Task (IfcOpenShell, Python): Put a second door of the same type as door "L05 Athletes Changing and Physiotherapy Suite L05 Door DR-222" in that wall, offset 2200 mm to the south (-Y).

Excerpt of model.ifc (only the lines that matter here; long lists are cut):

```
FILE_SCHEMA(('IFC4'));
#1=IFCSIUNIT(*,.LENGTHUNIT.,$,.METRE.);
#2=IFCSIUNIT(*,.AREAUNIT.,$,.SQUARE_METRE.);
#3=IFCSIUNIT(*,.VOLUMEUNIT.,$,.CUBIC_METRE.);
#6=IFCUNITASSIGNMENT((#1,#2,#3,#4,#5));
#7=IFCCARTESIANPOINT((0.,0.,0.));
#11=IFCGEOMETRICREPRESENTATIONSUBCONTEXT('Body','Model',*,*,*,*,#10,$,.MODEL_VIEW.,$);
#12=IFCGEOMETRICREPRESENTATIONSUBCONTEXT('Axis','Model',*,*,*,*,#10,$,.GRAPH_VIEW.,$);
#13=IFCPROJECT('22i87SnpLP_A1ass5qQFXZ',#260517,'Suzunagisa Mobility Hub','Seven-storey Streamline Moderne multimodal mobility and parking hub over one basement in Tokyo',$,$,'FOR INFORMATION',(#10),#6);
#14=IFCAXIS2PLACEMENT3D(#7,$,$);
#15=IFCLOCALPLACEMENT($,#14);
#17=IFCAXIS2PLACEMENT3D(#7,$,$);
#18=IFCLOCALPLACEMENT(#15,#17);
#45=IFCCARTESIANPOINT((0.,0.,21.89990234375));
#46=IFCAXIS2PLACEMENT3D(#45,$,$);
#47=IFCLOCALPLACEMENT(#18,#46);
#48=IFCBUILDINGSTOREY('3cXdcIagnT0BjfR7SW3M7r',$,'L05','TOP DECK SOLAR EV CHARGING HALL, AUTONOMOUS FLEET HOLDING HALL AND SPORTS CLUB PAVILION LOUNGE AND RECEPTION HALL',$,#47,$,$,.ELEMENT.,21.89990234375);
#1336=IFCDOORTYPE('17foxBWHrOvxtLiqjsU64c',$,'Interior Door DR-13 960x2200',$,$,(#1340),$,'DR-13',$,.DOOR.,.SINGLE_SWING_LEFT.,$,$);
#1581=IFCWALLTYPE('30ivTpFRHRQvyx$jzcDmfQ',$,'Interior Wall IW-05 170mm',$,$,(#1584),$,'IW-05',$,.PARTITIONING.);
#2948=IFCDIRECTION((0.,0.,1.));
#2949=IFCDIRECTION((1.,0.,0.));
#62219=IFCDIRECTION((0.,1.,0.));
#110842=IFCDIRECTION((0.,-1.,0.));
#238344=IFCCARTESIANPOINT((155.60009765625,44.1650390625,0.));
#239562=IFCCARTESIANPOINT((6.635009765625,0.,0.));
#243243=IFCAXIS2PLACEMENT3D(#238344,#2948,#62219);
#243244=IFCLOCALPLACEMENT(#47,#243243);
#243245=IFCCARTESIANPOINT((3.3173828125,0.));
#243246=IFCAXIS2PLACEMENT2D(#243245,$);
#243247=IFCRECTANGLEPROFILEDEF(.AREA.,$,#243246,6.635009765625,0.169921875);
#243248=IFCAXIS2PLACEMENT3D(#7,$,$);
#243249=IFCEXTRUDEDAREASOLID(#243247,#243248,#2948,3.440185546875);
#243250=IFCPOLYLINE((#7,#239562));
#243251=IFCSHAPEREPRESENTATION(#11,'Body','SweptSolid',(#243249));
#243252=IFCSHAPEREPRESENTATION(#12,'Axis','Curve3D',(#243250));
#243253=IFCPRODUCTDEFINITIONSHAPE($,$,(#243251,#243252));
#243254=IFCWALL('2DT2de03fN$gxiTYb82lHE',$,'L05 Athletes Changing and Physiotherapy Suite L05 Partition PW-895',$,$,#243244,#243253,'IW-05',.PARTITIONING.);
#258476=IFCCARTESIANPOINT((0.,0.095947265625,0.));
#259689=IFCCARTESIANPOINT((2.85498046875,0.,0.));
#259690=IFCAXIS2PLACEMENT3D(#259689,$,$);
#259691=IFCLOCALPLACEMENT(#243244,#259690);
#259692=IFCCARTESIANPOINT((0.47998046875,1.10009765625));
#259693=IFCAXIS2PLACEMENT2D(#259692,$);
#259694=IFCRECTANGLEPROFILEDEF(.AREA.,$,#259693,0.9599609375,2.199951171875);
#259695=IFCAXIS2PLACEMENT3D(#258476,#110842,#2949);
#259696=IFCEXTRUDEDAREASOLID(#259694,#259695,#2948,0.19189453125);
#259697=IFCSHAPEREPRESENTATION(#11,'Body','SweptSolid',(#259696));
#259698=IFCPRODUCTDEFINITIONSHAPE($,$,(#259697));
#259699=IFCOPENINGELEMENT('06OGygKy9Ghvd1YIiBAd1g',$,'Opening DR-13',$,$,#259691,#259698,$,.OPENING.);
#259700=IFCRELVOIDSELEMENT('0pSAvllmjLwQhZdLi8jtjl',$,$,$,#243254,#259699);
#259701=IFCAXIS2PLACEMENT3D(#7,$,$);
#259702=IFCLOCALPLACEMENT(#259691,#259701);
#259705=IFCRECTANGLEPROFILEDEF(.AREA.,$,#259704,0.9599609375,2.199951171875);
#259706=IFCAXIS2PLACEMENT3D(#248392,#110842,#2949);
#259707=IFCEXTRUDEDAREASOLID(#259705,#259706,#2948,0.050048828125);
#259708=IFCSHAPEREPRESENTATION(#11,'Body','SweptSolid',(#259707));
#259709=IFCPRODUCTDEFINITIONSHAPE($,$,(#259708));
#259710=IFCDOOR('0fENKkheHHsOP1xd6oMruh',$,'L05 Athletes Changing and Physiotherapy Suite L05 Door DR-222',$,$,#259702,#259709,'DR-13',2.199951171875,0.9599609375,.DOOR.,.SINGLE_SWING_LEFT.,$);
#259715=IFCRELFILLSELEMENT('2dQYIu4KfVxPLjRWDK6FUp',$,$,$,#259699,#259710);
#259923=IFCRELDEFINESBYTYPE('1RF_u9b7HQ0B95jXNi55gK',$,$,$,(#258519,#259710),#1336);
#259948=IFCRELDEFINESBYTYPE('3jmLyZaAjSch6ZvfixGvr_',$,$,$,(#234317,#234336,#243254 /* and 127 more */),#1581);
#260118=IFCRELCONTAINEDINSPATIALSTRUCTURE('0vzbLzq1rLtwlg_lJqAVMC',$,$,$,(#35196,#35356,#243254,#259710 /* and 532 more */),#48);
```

```python
import ifcopenshell
import ifcopenshell.api.feature
import ifcopenshell.api.geometry
import ifcopenshell.api.root
import ifcopenshell.geom
import ifcopenshell.util.element
import ifcopenshell.util.placement
import ifcopenshell.util.shape

model = ifcopenshell.open("model.ifc")
settings = ifcopenshell.geom.settings()


def volume(element):
    """Net volume in cubic metres, openings subtracted."""
    shape = ifcopenshell.geom.create_shape(settings, element)
    return ifcopenshell.util.shape.get_volume(shape.geometry)


door = model.by_guid("0fENKkheHHsOP1xd6oMruh")
opening = door.FillsVoids[0].RelatingOpeningElement
wall = opening.VoidsElements[0].RelatingBuildingElement
before = volume(wall)
shift = ifcopenshell.util.placement.get_local_placement(wall.ObjectPlacement)[:3, 0] * -2.2

# copy_class copies the void relationship, type, container and properties, but no geometry.
new_opening = ifcopenshell.api.root.copy_class(model, product=opening)
new_opening.Representation = ifcopenshell.util.element.copy_deep(
    model, opening.Representation, exclude=["IfcGeometricRepresentationContext", "IfcRepresentationMap"]
)
new_door = ifcopenshell.api.root.copy_class(model, product=door)
new_door.Representation = ifcopenshell.util.element.copy_deep(
    model, door.Representation, exclude=["IfcGeometricRepresentationContext", "IfcRepresentationMap"]
)
new_door.Tag = None
ifcopenshell.api.feature.add_filling(model, opening=new_opening, element=new_door)

for old, new in ((opening, new_opening), (door, new_door)):
    matrix = ifcopenshell.util.placement.get_local_placement(old.ObjectPlacement)
    matrix[:3, 3] += shift
    ifcopenshell.api.geometry.edit_object_placement(model, product=new, matrix=matrix, is_si=False)

after = volume(wall)

print(f"wall volume {before:.3f} -> {after:.3f} m3")

model.write("model_rev.ifc")
```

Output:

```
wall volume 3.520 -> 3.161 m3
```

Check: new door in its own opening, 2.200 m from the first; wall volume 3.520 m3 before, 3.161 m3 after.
